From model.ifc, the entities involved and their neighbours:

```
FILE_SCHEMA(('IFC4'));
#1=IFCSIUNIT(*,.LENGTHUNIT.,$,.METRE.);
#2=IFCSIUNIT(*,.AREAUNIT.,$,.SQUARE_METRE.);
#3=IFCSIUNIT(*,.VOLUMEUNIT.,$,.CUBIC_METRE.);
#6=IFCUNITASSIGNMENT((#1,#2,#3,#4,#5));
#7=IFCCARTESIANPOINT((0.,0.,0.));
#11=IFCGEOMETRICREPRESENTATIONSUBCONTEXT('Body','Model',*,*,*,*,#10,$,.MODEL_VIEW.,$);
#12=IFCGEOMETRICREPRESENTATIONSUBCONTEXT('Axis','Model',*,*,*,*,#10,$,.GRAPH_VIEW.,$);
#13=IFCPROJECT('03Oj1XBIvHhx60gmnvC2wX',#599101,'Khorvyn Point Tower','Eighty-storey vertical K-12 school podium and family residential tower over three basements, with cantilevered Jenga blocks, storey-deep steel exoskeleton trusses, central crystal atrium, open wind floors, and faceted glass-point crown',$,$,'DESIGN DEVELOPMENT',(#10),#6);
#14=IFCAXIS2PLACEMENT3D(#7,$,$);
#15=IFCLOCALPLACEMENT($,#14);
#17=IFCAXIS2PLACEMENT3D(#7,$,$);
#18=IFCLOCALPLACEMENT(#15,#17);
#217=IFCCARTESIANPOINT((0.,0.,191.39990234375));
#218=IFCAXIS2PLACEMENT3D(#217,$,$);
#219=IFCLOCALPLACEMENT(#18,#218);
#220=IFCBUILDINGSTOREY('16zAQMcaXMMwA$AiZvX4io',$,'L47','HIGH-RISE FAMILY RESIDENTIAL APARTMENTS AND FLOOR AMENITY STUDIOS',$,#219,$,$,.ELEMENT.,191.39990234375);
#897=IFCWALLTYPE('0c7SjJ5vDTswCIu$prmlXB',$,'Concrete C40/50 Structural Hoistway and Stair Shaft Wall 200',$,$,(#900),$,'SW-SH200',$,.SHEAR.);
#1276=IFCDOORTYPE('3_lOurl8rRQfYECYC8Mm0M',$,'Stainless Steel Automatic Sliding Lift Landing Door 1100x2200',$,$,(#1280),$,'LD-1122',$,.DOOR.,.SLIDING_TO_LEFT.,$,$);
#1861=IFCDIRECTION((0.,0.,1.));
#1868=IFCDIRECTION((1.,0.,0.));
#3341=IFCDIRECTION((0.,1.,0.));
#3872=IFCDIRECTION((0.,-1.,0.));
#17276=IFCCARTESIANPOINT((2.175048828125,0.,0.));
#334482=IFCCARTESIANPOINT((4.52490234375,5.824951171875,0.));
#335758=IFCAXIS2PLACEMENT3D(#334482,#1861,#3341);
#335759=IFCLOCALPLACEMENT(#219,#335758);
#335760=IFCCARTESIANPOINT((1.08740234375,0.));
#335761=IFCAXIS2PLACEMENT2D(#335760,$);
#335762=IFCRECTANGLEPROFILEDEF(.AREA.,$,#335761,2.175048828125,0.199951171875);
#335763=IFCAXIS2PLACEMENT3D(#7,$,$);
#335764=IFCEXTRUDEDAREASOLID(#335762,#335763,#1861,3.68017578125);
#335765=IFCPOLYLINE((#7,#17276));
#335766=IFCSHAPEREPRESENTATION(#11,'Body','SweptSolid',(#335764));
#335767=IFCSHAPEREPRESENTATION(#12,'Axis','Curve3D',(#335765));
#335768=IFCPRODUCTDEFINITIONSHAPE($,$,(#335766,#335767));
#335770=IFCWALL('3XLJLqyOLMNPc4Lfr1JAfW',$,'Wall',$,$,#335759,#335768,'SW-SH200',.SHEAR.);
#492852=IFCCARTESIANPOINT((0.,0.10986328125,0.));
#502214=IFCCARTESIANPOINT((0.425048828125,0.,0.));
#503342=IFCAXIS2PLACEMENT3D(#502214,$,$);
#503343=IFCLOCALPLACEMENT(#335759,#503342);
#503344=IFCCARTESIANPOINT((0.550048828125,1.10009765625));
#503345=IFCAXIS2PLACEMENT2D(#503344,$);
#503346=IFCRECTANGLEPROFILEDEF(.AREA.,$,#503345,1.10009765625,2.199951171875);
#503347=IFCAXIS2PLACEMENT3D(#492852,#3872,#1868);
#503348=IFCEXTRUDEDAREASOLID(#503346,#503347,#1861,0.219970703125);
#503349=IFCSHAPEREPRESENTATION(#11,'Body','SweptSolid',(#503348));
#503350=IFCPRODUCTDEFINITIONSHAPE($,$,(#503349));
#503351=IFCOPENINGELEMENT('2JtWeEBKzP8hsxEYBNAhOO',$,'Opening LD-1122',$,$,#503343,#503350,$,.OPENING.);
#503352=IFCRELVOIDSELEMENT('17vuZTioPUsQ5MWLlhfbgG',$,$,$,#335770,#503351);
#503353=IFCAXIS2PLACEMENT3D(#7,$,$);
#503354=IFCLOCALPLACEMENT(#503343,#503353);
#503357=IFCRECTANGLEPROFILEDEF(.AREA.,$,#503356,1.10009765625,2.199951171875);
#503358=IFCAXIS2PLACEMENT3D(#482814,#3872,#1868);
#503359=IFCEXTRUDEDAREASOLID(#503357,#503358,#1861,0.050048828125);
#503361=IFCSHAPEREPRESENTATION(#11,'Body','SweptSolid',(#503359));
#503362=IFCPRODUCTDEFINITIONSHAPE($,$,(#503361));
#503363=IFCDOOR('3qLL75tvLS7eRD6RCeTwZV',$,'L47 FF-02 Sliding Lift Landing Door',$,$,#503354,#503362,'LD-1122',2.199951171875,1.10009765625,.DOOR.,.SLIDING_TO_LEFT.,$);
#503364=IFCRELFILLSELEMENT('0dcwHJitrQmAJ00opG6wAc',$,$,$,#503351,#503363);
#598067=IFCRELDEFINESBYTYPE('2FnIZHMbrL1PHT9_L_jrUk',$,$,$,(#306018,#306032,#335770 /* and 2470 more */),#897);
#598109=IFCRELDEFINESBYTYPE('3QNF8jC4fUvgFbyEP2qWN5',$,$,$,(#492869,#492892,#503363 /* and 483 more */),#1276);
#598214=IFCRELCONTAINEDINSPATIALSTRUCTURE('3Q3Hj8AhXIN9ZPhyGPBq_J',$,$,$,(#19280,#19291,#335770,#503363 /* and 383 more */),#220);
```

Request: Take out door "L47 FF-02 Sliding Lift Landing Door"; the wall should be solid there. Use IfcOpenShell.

```python
import ifcopenshell
import ifcopenshell.api.feature
import ifcopenshell.api.root
import ifcopenshell.geom
import ifcopenshell.util.shape

model = ifcopenshell.open("model.ifc")
settings = ifcopenshell.geom.settings()


def volume(element):
    """Net volume in cubic metres, openings subtracted."""
    shape = ifcopenshell.geom.create_shape(settings, element)
    return ifcopenshell.util.shape.get_volume(shape.geometry)


door = model.by_guid("3qLL75tvLS7eRD6RCeTwZV")
opening = door.FillsVoids[0].RelatingOpeningElement
wall = opening.VoidsElements[0].RelatingBuildingElement
before = volume(wall)

ifcopenshell.api.root.remove_product(model, product=door)
ifcopenshell.api.feature.remove_feature(model, feature=opening)

after = volume(wall)

print(f"wall volume {before:.3f} -> {after:.3f} m3")

model.write("model_rev.ifc")
```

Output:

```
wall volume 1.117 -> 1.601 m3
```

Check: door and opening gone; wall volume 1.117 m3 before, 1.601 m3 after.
